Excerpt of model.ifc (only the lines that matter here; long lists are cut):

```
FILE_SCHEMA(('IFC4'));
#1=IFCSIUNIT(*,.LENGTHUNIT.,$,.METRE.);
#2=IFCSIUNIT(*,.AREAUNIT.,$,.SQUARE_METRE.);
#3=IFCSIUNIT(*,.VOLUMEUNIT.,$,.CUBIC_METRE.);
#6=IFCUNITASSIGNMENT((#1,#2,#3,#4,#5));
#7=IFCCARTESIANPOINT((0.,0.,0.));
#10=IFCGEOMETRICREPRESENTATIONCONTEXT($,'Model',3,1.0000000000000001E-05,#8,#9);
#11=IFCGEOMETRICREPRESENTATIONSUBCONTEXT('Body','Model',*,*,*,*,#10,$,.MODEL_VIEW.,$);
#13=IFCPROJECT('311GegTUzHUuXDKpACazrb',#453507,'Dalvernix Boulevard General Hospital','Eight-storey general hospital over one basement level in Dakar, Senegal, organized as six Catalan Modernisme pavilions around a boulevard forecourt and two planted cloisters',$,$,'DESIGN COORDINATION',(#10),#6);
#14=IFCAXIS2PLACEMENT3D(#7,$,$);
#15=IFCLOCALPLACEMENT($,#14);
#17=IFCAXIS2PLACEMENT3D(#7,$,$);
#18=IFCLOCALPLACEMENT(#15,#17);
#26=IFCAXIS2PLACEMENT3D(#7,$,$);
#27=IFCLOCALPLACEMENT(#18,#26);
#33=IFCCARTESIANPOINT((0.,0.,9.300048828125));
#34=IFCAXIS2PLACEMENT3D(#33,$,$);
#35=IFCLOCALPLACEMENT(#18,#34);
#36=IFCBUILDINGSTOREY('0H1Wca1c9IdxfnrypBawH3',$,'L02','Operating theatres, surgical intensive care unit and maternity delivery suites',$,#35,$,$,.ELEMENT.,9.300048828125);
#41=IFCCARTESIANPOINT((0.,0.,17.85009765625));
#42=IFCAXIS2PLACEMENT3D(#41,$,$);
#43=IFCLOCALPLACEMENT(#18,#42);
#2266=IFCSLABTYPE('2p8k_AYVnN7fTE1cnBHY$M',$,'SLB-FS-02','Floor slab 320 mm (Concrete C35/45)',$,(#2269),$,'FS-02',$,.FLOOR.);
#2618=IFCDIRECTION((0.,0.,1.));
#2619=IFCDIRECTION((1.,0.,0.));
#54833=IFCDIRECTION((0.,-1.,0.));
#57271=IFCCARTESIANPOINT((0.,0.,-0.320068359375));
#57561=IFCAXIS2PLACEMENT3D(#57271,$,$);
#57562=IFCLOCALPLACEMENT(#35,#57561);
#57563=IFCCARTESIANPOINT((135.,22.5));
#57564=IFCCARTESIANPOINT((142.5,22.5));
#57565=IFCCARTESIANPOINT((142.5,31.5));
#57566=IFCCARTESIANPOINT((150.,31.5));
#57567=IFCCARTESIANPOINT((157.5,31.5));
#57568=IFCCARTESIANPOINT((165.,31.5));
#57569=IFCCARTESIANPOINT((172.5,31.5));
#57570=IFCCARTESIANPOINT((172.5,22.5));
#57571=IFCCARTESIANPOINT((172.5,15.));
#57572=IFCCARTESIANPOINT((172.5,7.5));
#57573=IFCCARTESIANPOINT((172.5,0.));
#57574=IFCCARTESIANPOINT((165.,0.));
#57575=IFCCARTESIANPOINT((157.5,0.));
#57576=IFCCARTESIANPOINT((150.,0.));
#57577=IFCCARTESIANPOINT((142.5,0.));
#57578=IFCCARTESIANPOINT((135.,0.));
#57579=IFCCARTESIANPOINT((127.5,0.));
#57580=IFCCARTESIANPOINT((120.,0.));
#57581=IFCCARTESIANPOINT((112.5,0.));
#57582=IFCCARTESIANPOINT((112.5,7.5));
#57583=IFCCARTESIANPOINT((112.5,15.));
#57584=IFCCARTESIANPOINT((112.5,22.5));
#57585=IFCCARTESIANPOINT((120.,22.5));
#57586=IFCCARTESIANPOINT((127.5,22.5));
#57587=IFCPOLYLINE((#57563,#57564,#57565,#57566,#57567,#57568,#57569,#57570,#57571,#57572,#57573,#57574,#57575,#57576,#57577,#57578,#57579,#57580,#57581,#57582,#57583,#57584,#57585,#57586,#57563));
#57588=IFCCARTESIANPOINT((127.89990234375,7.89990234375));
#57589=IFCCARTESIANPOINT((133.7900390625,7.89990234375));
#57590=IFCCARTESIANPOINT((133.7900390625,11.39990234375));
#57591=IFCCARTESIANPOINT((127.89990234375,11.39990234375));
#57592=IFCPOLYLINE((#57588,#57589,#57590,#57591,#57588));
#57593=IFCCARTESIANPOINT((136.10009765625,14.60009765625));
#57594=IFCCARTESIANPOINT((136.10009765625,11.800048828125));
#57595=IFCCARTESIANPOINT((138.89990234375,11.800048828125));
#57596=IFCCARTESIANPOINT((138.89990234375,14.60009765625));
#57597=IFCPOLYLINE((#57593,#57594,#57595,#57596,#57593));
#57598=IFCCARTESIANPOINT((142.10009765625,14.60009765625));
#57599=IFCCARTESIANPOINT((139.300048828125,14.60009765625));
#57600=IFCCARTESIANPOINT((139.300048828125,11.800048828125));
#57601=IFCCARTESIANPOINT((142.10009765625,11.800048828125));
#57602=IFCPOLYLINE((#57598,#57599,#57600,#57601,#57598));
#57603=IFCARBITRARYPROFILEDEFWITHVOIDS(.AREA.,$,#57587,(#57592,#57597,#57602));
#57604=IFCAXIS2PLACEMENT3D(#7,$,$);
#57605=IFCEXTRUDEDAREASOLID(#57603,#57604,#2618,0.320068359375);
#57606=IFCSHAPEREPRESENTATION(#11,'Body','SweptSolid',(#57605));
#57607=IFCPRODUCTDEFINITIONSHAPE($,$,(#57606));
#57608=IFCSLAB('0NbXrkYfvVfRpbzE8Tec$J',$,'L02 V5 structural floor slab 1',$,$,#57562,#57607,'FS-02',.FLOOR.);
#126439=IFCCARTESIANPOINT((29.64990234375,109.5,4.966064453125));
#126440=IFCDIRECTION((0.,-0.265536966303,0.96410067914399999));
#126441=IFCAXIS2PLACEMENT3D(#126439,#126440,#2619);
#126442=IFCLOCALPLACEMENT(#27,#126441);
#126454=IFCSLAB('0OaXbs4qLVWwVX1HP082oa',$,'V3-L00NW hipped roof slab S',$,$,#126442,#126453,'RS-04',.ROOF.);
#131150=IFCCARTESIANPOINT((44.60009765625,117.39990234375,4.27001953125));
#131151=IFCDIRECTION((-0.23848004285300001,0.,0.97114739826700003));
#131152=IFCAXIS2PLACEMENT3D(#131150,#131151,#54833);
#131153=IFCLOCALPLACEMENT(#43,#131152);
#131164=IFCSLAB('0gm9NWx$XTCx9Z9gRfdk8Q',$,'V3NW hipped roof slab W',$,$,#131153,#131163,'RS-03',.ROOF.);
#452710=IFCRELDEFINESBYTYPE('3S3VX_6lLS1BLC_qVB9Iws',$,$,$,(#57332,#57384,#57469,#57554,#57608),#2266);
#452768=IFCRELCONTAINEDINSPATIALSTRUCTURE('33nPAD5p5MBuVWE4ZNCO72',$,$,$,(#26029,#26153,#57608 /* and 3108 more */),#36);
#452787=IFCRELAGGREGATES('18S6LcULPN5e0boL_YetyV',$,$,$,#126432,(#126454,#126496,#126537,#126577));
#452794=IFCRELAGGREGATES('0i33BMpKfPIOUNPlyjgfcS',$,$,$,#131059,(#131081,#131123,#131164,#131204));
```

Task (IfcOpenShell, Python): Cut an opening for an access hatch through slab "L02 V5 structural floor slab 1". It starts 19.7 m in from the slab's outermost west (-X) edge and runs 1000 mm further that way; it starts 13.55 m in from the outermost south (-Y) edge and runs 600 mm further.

```python
import numpy as np
import ifcopenshell
import ifcopenshell.api.feature
import ifcopenshell.api.geometry
import ifcopenshell.api.root
import ifcopenshell.geom
import ifcopenshell.util.placement
import ifcopenshell.util.representation
import ifcopenshell.util.shape
import ifcopenshell.util.unit

model = ifcopenshell.open("model.ifc")
unit_scale = ifcopenshell.util.unit.calculate_unit_scale(model)
settings = ifcopenshell.geom.settings()


def volume(element):
    """Net volume in cubic metres, openings subtracted."""
    shape = ifcopenshell.geom.create_shape(settings, element)
    return ifcopenshell.util.shape.get_volume(shape.geometry)


slab = model.by_guid("0NbXrkYfvVfRpbzE8Tec$J")
before = volume(slab)

# Extent in the slab's own axes, in metres. The edges named are its -X and -Y sides.
slab_shape = ifcopenshell.geom.create_shape(settings, slab)
vertices = ifcopenshell.util.shape.get_vertices(slab_shape.geometry)
x_min, y_min, bottom = vertices.min(axis=0)
top = vertices[:, 2].max()

opening = ifcopenshell.api.root.create_entity(model, ifc_class="IfcOpeningElement", name="Access hatch opening", predefined_type="OPENING")
context = ifcopenshell.util.representation.get_context(model, "Model", "Body", "MODEL_VIEW")
width, depth = 1, 0.6
outline = [(0.0, 0.0), (width, 0.0), (width, depth), (0.0, depth), (0.0, 0.0)]
# Overshoot both faces by 50 mm so the cut is clean.
shape = ifcopenshell.api.geometry.add_slab_representation(
    model, context=context, depth=top - bottom + 0.1, polyline=outline
)
ifcopenshell.api.geometry.assign_representation(model, product=opening, representation=shape)

matrix = ifcopenshell.util.placement.get_local_placement(slab.ObjectPlacement)
matrix[:, 3] = matrix @ np.append(np.array([x_min + 19.7, y_min + 13.55, bottom - 0.05]) / unit_scale, 1.0)
ifcopenshell.api.geometry.edit_object_placement(model, product=opening, matrix=matrix, is_si=False)
ifcopenshell.api.feature.add_feature(model, feature=opening, element=slab)

after = volume(slab)

print(f"slab volume {before:.3f} -> {after:.3f} m3")

model.write("model_updated.ifc")
```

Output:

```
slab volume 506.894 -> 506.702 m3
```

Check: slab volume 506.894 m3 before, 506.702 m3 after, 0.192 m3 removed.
